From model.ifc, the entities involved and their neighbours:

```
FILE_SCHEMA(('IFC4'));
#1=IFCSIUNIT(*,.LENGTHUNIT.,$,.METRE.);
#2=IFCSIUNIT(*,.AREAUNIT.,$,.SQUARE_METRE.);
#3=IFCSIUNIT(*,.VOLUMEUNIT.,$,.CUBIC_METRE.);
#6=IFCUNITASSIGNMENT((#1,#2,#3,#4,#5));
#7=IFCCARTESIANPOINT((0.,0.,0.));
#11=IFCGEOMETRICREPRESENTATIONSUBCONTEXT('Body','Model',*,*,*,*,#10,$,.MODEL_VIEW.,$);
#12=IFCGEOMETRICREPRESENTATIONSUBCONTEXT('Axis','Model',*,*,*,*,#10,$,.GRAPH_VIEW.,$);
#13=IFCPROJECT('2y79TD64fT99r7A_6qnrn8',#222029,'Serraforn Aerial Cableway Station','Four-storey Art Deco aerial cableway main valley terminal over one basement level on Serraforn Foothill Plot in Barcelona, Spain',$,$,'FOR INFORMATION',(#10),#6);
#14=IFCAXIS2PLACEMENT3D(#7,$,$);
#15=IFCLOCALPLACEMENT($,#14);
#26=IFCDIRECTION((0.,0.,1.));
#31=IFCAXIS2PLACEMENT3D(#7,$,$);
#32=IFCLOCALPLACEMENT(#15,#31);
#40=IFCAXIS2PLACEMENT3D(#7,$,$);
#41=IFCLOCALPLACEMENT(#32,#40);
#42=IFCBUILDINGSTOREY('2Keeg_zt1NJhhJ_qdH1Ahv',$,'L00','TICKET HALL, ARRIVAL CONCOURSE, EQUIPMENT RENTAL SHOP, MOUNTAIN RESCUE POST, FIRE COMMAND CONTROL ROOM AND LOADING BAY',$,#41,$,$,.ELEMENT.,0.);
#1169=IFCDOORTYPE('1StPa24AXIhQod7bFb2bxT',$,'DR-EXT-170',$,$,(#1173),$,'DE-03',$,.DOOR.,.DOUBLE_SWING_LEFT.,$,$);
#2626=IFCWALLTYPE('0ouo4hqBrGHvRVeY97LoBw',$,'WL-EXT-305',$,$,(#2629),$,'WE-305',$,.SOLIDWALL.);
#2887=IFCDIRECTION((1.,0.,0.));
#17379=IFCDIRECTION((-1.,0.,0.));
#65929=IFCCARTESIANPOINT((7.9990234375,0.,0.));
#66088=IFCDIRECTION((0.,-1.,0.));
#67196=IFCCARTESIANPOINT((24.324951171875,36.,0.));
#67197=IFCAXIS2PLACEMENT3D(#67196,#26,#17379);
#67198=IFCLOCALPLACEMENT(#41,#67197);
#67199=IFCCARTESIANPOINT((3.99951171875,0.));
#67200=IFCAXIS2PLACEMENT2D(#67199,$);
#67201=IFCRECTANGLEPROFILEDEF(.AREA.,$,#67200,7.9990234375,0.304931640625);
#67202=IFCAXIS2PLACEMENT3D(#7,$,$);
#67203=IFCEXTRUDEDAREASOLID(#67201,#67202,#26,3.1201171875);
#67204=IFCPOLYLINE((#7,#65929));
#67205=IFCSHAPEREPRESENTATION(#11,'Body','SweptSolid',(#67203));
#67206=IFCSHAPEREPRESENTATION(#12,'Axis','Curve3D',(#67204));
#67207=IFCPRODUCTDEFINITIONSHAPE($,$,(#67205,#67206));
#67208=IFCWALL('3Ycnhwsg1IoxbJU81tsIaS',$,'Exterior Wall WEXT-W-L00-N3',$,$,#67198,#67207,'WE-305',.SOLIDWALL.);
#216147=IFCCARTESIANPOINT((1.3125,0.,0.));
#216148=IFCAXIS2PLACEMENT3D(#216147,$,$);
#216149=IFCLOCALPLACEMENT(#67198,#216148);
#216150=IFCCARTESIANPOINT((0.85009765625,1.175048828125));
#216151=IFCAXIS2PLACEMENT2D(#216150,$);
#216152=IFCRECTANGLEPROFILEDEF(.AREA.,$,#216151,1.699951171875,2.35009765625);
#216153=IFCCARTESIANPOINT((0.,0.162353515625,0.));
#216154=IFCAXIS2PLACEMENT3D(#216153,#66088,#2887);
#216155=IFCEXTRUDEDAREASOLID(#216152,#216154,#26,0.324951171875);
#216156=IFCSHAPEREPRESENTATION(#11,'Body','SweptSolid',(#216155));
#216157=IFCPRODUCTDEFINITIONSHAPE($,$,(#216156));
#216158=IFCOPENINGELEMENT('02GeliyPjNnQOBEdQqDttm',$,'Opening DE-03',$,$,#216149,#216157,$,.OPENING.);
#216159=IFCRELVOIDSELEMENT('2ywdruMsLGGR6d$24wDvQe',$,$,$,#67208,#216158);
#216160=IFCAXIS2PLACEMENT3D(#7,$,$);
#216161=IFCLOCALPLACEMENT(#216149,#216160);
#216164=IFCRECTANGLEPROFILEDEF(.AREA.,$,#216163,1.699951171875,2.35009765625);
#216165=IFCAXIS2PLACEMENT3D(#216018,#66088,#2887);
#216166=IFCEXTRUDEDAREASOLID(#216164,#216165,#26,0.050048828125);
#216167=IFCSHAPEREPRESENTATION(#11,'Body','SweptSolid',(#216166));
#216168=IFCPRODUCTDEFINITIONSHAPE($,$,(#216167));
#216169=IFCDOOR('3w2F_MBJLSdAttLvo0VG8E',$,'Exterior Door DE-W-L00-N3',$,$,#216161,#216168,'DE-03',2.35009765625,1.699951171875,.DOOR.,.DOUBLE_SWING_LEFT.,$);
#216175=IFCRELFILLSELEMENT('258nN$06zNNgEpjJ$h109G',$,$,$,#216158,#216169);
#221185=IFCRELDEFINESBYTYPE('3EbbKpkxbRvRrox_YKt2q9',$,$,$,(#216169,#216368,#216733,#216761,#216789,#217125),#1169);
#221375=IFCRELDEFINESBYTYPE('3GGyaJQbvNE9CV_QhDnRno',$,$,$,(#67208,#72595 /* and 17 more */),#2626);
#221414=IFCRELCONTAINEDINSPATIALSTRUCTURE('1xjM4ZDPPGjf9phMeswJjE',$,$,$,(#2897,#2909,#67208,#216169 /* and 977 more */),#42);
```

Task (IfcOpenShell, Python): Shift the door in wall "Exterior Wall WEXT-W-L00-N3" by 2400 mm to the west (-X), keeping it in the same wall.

```python
import ifcopenshell
import ifcopenshell.api.geometry
import ifcopenshell.util.placement
import ifcopenshell.util.unit

model = ifcopenshell.open("model.ifc")
unit_scale = ifcopenshell.util.unit.calculate_unit_scale(model)

door = model.by_guid("3w2F_MBJLSdAttLvo0VG8E")
opening = door.FillsVoids[0].RelatingOpeningElement
wall = opening.VoidsElements[0].RelatingBuildingElement

wall_matrix = ifcopenshell.util.placement.get_local_placement(wall.ObjectPlacement)
shift = wall_matrix[:3, 0] * 2.4 / unit_scale
before = ifcopenshell.util.placement.get_local_placement(door.ObjectPlacement)[:3, 3].copy()

# The door is placed relative to its opening, so it follows when the opening moves.
matrix = ifcopenshell.util.placement.get_local_placement(opening.ObjectPlacement)
matrix[:3, 3] += shift
ifcopenshell.api.geometry.edit_object_placement(
    model, product=opening, matrix=matrix, is_si=False, should_transform_children=True
)

after = ifcopenshell.util.placement.get_local_placement(door.ObjectPlacement)[:3, 3]
print("door moved by", (after - before).round(3) + 0.0)

model.write("model_edited.ifc")
```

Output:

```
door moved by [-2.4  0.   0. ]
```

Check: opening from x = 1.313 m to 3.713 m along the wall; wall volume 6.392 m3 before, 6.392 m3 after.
